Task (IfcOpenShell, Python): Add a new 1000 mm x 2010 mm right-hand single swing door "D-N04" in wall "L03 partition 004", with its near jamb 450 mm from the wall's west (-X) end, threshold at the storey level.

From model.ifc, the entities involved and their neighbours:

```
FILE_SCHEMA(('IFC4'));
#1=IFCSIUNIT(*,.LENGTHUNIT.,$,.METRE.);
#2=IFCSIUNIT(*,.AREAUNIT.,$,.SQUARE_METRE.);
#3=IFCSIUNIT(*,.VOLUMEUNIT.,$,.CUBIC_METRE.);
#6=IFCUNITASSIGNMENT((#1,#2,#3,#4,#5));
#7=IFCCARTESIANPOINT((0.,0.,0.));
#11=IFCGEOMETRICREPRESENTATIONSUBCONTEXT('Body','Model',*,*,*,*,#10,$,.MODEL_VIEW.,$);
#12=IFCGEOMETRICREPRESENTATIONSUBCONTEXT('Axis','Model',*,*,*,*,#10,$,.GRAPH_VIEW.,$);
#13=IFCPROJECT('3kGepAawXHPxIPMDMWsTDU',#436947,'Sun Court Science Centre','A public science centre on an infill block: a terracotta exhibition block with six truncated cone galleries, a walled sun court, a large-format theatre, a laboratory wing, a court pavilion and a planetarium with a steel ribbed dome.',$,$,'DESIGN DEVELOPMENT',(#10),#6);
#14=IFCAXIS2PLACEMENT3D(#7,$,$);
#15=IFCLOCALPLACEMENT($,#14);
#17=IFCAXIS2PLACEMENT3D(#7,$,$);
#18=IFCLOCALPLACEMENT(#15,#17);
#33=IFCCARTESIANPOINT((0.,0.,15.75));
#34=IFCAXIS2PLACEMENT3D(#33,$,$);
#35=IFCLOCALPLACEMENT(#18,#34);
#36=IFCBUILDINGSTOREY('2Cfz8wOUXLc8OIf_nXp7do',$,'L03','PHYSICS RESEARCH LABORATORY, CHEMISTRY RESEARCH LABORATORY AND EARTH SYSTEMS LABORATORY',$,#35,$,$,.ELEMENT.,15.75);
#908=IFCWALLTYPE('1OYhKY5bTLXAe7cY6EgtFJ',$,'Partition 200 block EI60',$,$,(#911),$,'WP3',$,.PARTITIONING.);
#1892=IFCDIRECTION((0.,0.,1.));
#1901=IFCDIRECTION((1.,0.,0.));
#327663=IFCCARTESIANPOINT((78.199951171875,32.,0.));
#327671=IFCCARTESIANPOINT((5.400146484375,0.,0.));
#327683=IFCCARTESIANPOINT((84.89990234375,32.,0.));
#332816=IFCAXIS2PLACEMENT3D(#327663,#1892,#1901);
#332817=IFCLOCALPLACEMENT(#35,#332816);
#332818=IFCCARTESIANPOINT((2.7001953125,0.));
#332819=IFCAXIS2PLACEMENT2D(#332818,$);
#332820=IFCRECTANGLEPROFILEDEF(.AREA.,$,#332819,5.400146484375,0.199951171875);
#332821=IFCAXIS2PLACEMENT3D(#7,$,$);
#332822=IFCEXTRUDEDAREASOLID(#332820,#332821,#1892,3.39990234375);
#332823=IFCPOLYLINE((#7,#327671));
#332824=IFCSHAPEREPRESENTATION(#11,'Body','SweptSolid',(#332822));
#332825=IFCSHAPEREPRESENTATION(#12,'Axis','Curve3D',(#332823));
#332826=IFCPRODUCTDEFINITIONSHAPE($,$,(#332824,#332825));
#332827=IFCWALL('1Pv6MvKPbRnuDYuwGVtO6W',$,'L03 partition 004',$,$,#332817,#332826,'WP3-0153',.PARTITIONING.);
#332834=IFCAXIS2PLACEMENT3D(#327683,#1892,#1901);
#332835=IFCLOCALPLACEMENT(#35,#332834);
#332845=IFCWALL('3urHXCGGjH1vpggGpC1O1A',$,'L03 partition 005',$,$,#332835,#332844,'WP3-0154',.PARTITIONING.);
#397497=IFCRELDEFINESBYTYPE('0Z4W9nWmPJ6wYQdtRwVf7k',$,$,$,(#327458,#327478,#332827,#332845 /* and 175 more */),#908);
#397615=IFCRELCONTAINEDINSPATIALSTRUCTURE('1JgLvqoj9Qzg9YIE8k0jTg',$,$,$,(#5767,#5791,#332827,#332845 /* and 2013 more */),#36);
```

```python
import numpy as np
import ifcopenshell
import ifcopenshell.api.feature
import ifcopenshell.api.geometry
import ifcopenshell.api.root
import ifcopenshell.api.spatial
import ifcopenshell.geom
import ifcopenshell.util.element
import ifcopenshell.util.placement
import ifcopenshell.util.representation
import ifcopenshell.util.shape
import ifcopenshell.util.unit

model = ifcopenshell.open("model.ifc")
unit_scale = ifcopenshell.util.unit.calculate_unit_scale(model)
settings = ifcopenshell.geom.settings()


def volume(element):
    """Net volume in cubic metres, openings subtracted."""
    shape = ifcopenshell.geom.create_shape(settings, element)
    return ifcopenshell.util.shape.get_volume(shape.geometry)


wall = model.by_id(332827)
storey = ifcopenshell.util.element.get_container(wall, ifc_class="IfcBuildingStorey")
context = ifcopenshell.util.representation.get_context(model, "Model", "Body", "MODEL_VIEW")
before = volume(wall)

width, height, from_end, sill = 1, 2.01, 0.45, 0.0  # metres

# The wall runs along its own X axis, and the end named is its -X end.
wall_shape = ifcopenshell.geom.create_shape(settings, wall)
x, y, z = ifcopenshell.util.shape.get_vertices(wall_shape.geometry).T
start = x.min() + from_end
face, thickness = float(y.min()), float(y.max() - y.min())
wall_matrix = ifcopenshell.util.placement.get_local_placement(wall.ObjectPlacement)
level = ifcopenshell.util.placement.get_local_placement(storey.ObjectPlacement)[2, 3]


def in_wall(x, y):
    """Placement at x, y metres in the wall's axes, at sill height."""
    matrix = wall_matrix.copy()
    matrix[:, 3] = wall_matrix @ np.array([x / unit_scale, y / unit_scale, 0.0, 1.0])
    matrix[2, 3] = level + sill / unit_scale
    return matrix


# Opening: a box that overshoots both wall faces by 50 mm.
opening = ifcopenshell.api.root.create_entity(model, ifc_class="IfcOpeningElement", predefined_type="OPENING")
box = ifcopenshell.api.geometry.add_wall_representation(
    model, context=context, length=width, height=height, thickness=thickness + 0.1
)
ifcopenshell.api.geometry.assign_representation(model, product=opening, representation=box)
ifcopenshell.api.geometry.edit_object_placement(model, product=opening, matrix=in_wall(start, face - 0.05), is_si=False)
ifcopenshell.api.feature.add_feature(model, feature=opening, element=wall)

door = ifcopenshell.api.root.create_entity(model, ifc_class="IfcDoor", name="D-N04", predefined_type="DOOR")
door.OverallWidth, door.OverallHeight = width / unit_scale, height / unit_scale
door.OperationType = "SINGLE_SWING_RIGHT"
body = ifcopenshell.api.geometry.add_door_representation(
    model,
    context=context,
    overall_width=door.OverallWidth,
    overall_height=door.OverallHeight,
    operation_type="SINGLE_SWING_RIGHT",
    lining_properties={"LiningDepth": thickness / unit_scale, "ThresholdDepth": thickness / unit_scale},
)
ifcopenshell.api.geometry.assign_representation(model, product=door, representation=body)
ifcopenshell.api.spatial.assign_container(model, products=[door], relating_structure=storey)
ifcopenshell.api.feature.add_filling(model, opening=opening, element=door)

# The lining spans the wall, so the door starts at the wall face.
ifcopenshell.api.geometry.edit_object_placement(model, product=door, matrix=in_wall(start, face), is_si=False)

after = volume(wall)

print(f"wall volume {before:.3f} -> {after:.3f} m3")

model.write("model_updated.ifc")
```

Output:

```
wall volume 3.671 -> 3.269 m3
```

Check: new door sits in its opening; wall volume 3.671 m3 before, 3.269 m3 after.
